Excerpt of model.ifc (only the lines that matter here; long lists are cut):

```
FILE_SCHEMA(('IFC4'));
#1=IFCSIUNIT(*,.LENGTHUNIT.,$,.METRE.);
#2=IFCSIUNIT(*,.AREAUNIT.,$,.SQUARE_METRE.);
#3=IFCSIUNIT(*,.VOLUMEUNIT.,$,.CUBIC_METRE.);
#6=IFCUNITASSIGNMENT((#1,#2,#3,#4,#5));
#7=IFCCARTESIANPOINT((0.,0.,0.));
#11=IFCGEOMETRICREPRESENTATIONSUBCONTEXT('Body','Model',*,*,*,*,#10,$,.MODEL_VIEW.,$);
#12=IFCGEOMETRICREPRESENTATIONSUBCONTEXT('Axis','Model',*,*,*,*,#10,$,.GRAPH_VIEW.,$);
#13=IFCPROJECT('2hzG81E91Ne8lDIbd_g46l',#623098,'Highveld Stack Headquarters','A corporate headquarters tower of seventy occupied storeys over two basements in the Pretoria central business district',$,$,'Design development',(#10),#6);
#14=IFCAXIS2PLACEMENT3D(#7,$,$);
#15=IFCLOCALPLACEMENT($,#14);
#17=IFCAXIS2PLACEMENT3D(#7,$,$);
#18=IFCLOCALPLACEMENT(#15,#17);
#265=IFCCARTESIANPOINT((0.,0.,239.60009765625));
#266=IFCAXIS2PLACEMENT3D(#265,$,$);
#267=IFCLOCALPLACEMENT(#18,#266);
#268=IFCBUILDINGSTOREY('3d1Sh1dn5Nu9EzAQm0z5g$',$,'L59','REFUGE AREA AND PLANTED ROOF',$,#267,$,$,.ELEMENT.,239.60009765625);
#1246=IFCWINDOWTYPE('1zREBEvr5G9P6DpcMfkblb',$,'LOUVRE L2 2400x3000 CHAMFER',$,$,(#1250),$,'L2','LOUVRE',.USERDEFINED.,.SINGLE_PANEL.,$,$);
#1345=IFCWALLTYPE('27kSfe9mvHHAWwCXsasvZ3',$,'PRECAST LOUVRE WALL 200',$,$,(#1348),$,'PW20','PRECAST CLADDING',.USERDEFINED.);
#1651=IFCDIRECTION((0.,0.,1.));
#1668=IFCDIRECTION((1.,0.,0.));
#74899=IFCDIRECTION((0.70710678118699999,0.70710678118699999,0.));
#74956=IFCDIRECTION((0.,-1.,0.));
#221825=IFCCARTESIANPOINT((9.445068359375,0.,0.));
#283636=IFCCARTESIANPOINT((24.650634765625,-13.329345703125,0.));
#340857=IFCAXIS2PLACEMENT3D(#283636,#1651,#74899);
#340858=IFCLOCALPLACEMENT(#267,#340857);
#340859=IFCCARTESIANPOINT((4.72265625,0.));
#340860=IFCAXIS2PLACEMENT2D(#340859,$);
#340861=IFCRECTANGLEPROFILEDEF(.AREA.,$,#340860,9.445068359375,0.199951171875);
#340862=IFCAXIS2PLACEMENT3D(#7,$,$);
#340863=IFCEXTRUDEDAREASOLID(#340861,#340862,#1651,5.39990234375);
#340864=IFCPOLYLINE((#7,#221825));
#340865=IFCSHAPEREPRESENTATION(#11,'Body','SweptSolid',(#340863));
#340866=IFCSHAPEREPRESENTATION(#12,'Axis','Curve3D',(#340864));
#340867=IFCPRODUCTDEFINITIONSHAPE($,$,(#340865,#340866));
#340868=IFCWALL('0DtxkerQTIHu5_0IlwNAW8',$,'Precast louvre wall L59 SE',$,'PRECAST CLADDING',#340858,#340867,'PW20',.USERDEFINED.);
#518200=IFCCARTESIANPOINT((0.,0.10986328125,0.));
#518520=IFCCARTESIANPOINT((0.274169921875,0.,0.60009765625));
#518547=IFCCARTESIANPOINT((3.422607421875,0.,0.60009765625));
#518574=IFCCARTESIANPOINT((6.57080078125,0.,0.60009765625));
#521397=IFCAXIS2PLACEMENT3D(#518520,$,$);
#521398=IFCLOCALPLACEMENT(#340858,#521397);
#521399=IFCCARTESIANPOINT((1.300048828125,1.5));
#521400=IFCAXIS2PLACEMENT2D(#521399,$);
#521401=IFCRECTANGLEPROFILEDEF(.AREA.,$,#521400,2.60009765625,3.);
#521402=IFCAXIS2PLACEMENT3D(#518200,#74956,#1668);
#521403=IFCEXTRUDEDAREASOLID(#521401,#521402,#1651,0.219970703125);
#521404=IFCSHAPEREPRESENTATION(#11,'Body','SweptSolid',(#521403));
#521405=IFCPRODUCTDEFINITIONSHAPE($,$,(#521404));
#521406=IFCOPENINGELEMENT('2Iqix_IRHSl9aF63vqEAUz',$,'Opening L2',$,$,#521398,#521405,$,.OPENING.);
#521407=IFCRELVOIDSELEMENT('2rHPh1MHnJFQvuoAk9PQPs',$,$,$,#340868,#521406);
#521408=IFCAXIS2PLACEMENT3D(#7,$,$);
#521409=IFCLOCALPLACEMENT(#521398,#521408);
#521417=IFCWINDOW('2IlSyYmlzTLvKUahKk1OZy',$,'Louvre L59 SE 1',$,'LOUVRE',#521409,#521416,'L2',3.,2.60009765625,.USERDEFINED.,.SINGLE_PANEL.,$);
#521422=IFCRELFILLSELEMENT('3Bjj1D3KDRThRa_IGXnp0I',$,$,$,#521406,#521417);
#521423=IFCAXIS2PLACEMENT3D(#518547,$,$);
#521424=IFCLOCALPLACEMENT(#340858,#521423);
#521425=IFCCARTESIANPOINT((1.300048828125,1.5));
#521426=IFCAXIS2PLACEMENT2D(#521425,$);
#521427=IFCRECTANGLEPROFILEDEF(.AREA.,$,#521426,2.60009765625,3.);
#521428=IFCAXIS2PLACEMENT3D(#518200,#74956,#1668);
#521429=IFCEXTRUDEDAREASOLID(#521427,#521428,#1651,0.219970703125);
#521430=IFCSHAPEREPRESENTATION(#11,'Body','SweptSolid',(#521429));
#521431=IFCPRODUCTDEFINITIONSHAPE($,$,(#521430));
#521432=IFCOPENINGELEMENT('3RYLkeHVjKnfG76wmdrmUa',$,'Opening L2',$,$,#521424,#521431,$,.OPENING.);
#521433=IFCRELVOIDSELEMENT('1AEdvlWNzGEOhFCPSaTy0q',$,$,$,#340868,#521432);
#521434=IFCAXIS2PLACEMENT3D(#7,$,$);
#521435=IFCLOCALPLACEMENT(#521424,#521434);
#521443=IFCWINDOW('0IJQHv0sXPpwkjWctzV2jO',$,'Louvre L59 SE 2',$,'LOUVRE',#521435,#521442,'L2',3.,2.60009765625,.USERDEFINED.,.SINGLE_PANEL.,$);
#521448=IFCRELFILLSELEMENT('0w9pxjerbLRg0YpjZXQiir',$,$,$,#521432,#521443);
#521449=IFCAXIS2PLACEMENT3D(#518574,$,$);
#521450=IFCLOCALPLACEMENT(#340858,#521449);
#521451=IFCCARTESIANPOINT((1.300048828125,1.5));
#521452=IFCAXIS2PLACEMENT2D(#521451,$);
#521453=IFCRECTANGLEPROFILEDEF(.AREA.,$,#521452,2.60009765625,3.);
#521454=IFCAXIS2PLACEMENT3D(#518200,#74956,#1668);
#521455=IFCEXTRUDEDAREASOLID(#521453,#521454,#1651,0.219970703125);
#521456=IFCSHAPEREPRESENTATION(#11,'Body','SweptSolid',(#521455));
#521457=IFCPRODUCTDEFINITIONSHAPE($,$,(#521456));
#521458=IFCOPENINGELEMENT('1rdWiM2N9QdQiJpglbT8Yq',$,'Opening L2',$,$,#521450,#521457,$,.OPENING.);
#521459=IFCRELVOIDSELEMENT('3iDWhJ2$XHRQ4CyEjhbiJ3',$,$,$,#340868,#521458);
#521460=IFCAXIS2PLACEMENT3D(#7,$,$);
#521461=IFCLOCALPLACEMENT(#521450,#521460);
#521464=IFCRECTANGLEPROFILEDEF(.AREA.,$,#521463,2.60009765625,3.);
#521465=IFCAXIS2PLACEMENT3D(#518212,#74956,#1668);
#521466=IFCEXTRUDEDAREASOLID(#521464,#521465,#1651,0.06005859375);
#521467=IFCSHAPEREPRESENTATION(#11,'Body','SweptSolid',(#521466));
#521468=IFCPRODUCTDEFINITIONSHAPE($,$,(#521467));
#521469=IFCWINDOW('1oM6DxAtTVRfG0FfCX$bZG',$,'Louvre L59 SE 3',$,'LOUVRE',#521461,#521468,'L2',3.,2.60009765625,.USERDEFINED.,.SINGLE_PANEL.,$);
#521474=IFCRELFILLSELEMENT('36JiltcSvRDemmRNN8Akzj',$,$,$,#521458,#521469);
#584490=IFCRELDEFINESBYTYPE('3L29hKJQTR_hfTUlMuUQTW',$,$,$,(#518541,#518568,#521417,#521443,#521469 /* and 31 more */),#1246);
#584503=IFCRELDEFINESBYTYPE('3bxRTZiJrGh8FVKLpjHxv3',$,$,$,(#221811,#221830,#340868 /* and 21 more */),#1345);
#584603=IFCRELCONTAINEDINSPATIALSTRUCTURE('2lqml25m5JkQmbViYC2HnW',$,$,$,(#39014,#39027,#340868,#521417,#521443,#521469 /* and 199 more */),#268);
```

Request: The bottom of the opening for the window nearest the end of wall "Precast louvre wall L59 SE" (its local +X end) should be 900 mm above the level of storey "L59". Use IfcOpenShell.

```python
import numpy as np
import ifcopenshell
import ifcopenshell.api.geometry
import ifcopenshell.geom
import ifcopenshell.util.element
import ifcopenshell.util.placement
import ifcopenshell.util.shape
import ifcopenshell.util.unit

model = ifcopenshell.open("model.ifc")
unit_scale = ifcopenshell.util.unit.calculate_unit_scale(model)

window = model.by_id(521469)
opening = window.FillsVoids[0].RelatingOpeningElement
storey = ifcopenshell.util.element.get_container(window, ifc_class="IfcBuildingStorey")
level = ifcopenshell.util.placement.get_local_placement(storey.ObjectPlacement)[2, 3]

# The opening's origin need not be at the sill, so measure its lowest point.
shape = ifcopenshell.geom.create_shape(ifcopenshell.geom.settings(), opening)
bottom = ifcopenshell.util.shape.get_shape_bottom_elevation(shape, shape.geometry) / unit_scale
dz = level + 0.9 / unit_scale - bottom

shift = np.array([0.0, 0.0, dz])
# The window is placed relative to its opening, so it follows when the opening moves.
matrix = ifcopenshell.util.placement.get_local_placement(opening.ObjectPlacement)
matrix[:3, 3] += shift
ifcopenshell.api.geometry.edit_object_placement(
    model, product=opening, matrix=matrix, is_si=False, should_transform_children=True
)

print(f"moved by {dz * unit_scale:+.3f} m")

model.write("model_updated.ifc")
```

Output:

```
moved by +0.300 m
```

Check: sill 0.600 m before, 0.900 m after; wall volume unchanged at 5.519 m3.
